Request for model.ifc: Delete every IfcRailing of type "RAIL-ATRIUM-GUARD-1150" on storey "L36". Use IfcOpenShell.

First a look at what the model holds.

```python
import ifcopenshell
import ifcopenshell.util.element

model = ifcopenshell.open("model.ifc")
print(model.schema)
storey = next(s for s in model.by_type("IfcBuildingStorey") if s.Name == "L36")
railings = [e for e in ifcopenshell.util.element.get_decomposition(storey) if e.is_a("IfcRailing")]
seen = {}
for e in railings:
    element_type = ifcopenshell.util.element.get_type(e)
    name = element_type.Name if element_type not in (None, e) else None
    seen[name] = seen.get(name, 0) + 1
for name, count in sorted(seen.items(), key=str):
    print(count, "x", name)
```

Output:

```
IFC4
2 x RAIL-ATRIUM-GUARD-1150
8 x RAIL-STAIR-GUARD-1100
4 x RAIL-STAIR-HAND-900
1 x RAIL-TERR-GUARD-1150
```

```python
import ifcopenshell
import ifcopenshell.api.root
import ifcopenshell.util.element

model = ifcopenshell.open("model.ifc")

storey = next(s for s in model.by_type("IfcBuildingStorey") if s.Name == "L36")
railings = [e for e in ifcopenshell.util.element.get_decomposition(storey) if e.is_a("IfcRailing")]
targets = [e for e in railings if (t := ifcopenshell.util.element.get_type(e)) not in (None, e) and t.Name == "RAIL-ATRIUM-GUARD-1150"]

for e in targets:
    ifcopenshell.api.root.remove_product(model, product=e)
print(len(targets), "removed")

model.write("model_updated.ifc")
```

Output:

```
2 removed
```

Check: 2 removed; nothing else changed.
